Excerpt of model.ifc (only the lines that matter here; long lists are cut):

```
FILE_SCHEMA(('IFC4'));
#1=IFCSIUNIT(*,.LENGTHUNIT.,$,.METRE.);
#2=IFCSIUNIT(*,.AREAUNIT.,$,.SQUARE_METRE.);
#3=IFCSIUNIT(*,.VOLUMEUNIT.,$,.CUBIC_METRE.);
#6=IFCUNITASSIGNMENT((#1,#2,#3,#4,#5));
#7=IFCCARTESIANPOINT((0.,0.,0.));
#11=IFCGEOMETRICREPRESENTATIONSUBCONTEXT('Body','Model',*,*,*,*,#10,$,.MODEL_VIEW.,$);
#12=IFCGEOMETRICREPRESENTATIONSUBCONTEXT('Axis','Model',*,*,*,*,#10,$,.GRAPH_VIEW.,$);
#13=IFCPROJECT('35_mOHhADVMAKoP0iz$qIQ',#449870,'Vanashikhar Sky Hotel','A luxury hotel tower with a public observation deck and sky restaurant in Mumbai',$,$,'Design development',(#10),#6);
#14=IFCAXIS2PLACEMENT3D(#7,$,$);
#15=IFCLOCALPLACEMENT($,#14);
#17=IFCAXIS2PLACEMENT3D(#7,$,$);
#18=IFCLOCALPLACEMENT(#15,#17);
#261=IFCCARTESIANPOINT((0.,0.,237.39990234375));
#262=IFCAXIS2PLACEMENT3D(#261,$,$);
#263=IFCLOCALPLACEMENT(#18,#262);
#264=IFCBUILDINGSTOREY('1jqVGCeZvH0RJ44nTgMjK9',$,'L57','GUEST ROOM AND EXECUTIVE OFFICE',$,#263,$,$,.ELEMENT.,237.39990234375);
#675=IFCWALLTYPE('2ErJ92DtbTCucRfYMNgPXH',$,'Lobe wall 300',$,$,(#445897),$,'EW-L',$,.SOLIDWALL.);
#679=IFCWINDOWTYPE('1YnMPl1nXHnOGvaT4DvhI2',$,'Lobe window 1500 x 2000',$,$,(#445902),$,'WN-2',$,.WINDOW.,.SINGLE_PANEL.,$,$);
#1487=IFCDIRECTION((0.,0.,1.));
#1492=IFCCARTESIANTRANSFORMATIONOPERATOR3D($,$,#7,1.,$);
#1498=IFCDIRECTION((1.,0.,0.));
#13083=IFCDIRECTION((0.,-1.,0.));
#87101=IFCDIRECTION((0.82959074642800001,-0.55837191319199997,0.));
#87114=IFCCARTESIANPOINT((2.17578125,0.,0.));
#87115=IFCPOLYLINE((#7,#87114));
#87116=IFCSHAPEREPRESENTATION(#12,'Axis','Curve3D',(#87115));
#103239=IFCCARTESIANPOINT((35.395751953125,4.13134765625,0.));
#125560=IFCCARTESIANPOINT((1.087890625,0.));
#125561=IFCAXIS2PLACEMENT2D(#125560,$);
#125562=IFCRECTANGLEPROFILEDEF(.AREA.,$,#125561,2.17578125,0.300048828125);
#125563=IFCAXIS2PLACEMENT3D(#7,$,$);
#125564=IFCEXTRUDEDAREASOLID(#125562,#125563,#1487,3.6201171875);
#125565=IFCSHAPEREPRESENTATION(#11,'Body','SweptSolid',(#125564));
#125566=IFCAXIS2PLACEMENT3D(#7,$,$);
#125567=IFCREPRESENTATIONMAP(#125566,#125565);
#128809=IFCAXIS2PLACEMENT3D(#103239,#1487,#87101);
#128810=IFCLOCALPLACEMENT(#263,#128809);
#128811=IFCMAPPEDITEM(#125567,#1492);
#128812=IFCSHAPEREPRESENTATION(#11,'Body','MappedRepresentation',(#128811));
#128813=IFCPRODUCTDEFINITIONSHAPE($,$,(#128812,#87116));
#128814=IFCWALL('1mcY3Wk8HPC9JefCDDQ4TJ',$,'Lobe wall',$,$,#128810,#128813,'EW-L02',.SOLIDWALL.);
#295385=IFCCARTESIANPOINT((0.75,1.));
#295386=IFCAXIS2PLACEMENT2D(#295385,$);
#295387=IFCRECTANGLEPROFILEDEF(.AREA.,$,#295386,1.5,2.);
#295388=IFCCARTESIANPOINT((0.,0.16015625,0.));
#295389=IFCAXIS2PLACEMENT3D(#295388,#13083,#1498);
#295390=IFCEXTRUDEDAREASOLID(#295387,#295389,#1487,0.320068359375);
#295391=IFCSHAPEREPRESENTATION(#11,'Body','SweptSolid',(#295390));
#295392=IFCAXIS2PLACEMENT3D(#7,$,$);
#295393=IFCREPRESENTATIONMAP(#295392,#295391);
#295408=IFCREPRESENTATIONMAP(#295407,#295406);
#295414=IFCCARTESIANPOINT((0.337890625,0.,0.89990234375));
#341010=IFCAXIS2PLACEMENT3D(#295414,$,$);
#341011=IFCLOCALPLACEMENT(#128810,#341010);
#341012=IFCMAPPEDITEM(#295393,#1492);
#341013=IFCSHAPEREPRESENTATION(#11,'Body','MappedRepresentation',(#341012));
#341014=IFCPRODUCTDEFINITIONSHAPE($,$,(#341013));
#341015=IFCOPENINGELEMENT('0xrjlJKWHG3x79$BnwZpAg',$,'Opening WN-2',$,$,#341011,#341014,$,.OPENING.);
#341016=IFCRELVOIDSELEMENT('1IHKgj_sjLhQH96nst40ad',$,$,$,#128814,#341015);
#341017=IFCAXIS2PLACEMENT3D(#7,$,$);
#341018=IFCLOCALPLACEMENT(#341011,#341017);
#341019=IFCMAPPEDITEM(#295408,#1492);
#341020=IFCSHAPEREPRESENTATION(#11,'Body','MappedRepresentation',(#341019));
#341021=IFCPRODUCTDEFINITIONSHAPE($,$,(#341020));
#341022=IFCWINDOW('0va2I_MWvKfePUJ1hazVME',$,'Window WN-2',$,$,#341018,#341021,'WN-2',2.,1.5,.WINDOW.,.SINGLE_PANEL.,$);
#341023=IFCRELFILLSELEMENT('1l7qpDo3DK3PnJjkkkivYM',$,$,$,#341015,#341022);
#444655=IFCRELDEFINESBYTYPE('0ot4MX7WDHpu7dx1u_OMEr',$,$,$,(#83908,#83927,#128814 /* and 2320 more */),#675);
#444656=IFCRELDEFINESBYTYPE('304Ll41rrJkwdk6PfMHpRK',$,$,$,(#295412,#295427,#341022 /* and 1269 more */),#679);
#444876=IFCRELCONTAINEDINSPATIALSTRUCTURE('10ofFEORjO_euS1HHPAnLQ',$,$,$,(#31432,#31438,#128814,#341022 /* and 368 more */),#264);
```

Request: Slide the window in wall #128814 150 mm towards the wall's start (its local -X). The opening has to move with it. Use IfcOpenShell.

```python
import ifcopenshell
import ifcopenshell.api.geometry
import ifcopenshell.util.placement

model = ifcopenshell.open("model.ifc")

window = model.by_id(341022)
opening = window.FillsVoids[0].RelatingOpeningElement
wall = opening.VoidsElements[0].RelatingBuildingElement

wall_matrix = ifcopenshell.util.placement.get_local_placement(wall.ObjectPlacement)
shift = wall_matrix[:3, 0] * -0.15
before = ifcopenshell.util.placement.get_local_placement(window.ObjectPlacement)[:3, 3].copy()

# The window is placed relative to its opening, so it follows when the opening moves.
matrix = ifcopenshell.util.placement.get_local_placement(opening.ObjectPlacement)
matrix[:3, 3] += shift
ifcopenshell.api.geometry.edit_object_placement(
    model, product=opening, matrix=matrix, is_si=False, should_transform_children=True
)

after = ifcopenshell.util.placement.get_local_placement(window.ObjectPlacement)[:3, 3]
print("window moved by", (after - before).round(3) + 0.0)

model.write("model_updated.ifc")
```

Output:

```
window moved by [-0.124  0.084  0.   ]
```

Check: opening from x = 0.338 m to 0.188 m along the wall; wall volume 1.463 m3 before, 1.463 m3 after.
